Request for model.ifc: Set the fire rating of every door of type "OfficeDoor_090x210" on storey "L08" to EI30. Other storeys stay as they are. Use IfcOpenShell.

First a look at what the model holds.

```python
import ifcopenshell
import ifcopenshell.util.element

model = ifcopenshell.open("model.ifc")
print(model.schema)
storey = next(s for s in model.by_type("IfcBuildingStorey") if s.Name == "L08")
doors = [e for e in ifcopenshell.util.element.get_decomposition(storey) if e.is_a("IfcDoor")]
seen = {}
for e in doors:
    element_type = ifcopenshell.util.element.get_type(e)
    key = (element_type.Name if element_type != e and element_type else None, ifcopenshell.util.element.get_pset(e, "Pset_DoorCommon", "FireRating"))
    seen[key] = seen.get(key, 0) + 1
for (name, value), count in sorted(seen.items(), key=str):
    print(count, "x", name, "|", value)
```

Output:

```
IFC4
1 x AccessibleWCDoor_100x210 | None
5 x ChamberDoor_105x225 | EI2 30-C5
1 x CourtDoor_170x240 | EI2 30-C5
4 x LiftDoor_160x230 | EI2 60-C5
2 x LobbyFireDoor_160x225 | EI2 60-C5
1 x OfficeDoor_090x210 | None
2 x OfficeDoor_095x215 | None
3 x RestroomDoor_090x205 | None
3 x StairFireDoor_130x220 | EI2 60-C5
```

```python
import ifcopenshell
import ifcopenshell.api.pset
import ifcopenshell.util.element

model = ifcopenshell.open("model.ifc")

storey = next(s for s in model.by_type("IfcBuildingStorey") if s.Name == "L08")
doors = [e for e in ifcopenshell.util.element.get_decomposition(storey) if e.is_a("IfcDoor")]

count = 0
for e in doors:
    element_type = ifcopenshell.util.element.get_type(e)
    if element_type in (None, e) or element_type.Name != "OfficeDoor_090x210":
        continue
    # add_pset returns the element's existing set when there is one.
    pset = ifcopenshell.api.pset.add_pset(model, product=e, name="Pset_DoorCommon")
    ifcopenshell.api.pset.edit_pset(model, pset=pset, properties={"FireRating": "EI30"})
    count += 1

print(count, "doors updated")

model.write("model_v2.ifc")
```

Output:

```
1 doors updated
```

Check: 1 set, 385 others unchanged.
